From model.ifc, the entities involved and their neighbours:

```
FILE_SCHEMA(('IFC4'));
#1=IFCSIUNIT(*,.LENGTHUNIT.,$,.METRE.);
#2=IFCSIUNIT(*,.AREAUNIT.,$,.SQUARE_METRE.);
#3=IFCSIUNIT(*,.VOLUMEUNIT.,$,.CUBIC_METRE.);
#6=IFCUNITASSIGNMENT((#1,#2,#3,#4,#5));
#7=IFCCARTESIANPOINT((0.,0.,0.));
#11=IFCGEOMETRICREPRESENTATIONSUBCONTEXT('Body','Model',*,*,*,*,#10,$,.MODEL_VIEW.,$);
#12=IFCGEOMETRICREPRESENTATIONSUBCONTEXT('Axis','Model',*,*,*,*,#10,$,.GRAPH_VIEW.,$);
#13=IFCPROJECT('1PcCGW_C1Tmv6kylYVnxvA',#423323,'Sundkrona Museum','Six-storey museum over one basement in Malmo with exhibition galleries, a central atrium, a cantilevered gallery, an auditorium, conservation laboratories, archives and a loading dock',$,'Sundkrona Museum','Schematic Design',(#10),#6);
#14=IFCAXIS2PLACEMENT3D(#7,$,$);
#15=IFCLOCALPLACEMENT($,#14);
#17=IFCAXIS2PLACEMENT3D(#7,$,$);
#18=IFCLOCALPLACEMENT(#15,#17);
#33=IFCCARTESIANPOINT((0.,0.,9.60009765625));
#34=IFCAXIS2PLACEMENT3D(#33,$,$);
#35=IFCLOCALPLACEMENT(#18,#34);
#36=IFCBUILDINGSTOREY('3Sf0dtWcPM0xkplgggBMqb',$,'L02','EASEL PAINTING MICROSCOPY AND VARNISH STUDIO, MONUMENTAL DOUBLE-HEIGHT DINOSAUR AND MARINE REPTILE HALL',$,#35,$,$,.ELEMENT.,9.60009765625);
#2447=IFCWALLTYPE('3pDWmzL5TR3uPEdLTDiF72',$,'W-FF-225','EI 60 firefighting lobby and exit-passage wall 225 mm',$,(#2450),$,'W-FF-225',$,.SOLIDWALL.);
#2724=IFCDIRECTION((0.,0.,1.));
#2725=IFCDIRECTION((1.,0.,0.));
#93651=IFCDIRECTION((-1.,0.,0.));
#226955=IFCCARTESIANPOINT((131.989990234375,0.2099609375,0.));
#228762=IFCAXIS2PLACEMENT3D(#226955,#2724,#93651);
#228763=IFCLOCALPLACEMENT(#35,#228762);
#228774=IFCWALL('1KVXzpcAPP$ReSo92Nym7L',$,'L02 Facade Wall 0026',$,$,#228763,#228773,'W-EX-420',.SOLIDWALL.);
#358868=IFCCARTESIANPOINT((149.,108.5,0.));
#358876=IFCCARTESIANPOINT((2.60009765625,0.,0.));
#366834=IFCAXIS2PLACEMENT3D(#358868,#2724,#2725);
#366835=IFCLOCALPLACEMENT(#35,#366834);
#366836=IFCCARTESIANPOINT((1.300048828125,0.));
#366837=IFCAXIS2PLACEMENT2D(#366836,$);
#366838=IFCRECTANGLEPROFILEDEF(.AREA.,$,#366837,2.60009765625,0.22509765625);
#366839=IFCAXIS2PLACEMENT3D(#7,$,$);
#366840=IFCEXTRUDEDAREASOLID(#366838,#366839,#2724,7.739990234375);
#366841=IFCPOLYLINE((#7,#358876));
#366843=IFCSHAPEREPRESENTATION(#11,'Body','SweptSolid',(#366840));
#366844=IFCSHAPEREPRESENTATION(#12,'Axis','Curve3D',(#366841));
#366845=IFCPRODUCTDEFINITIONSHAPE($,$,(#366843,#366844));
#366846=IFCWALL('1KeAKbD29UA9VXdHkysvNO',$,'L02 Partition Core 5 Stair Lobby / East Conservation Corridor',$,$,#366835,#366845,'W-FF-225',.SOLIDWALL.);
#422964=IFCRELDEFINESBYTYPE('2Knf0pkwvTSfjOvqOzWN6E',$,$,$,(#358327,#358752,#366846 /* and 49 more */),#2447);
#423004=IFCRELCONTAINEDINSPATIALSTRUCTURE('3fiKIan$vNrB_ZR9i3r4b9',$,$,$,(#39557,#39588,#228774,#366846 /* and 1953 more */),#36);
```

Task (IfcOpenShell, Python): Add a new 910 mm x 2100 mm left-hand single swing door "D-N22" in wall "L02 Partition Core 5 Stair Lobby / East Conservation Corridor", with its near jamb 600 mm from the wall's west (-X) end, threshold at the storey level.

```python
import numpy as np
import ifcopenshell
import ifcopenshell.api.feature
import ifcopenshell.api.geometry
import ifcopenshell.api.root
import ifcopenshell.api.spatial
import ifcopenshell.geom
import ifcopenshell.util.element
import ifcopenshell.util.placement
import ifcopenshell.util.representation
import ifcopenshell.util.shape
import ifcopenshell.util.unit

model = ifcopenshell.open("model.ifc")
unit_scale = ifcopenshell.util.unit.calculate_unit_scale(model)
settings = ifcopenshell.geom.settings()


def volume(element):
    """Net volume in cubic metres, openings subtracted."""
    shape = ifcopenshell.geom.create_shape(settings, element)
    return ifcopenshell.util.shape.get_volume(shape.geometry)


wall = model.by_guid("1KeAKbD29UA9VXdHkysvNO")
storey = ifcopenshell.util.element.get_container(wall, ifc_class="IfcBuildingStorey")
context = ifcopenshell.util.representation.get_context(model, "Model", "Body", "MODEL_VIEW")
before = volume(wall)

width, height, from_end, sill = 0.91, 2.1, 0.6, 0.0  # metres

# The wall runs along its own X axis, and the end named is its -X end.
wall_shape = ifcopenshell.geom.create_shape(settings, wall)
x, y, z = ifcopenshell.util.shape.get_vertices(wall_shape.geometry).T
start = x.min() + from_end
face, thickness = float(y.min()), float(y.max() - y.min())
wall_matrix = ifcopenshell.util.placement.get_local_placement(wall.ObjectPlacement)
level = ifcopenshell.util.placement.get_local_placement(storey.ObjectPlacement)[2, 3]


def in_wall(x, y):
    """Placement at x, y metres in the wall's axes, at sill height."""
    matrix = wall_matrix.copy()
    matrix[:, 3] = wall_matrix @ np.array([x / unit_scale, y / unit_scale, 0.0, 1.0])
    matrix[2, 3] = level + sill / unit_scale
    return matrix


# Opening: a box that overshoots both wall faces by 50 mm.
opening = ifcopenshell.api.root.create_entity(model, ifc_class="IfcOpeningElement", predefined_type="OPENING")
box = ifcopenshell.api.geometry.add_wall_representation(
    model, context=context, length=width, height=height, thickness=thickness + 0.1
)
ifcopenshell.api.geometry.assign_representation(model, product=opening, representation=box)
ifcopenshell.api.geometry.edit_object_placement(model, product=opening, matrix=in_wall(start, face - 0.05), is_si=False)
ifcopenshell.api.feature.add_feature(model, feature=opening, element=wall)

door = ifcopenshell.api.root.create_entity(model, ifc_class="IfcDoor", name="D-N22", predefined_type="DOOR")
door.OverallWidth, door.OverallHeight = width / unit_scale, height / unit_scale
door.OperationType = "SINGLE_SWING_LEFT"
body = ifcopenshell.api.geometry.add_door_representation(
    model,
    context=context,
    overall_width=door.OverallWidth,
    overall_height=door.OverallHeight,
    operation_type="SINGLE_SWING_LEFT",
    lining_properties={"LiningDepth": thickness / unit_scale, "ThresholdDepth": thickness / unit_scale},
)
ifcopenshell.api.geometry.assign_representation(model, product=door, representation=body)
ifcopenshell.api.spatial.assign_container(model, products=[door], relating_structure=storey)
ifcopenshell.api.feature.add_filling(model, opening=opening, element=door)

# The lining spans the wall, so the door starts at the wall face.
ifcopenshell.api.geometry.edit_object_placement(model, product=door, matrix=in_wall(start, face), is_si=False)

after = volume(wall)

print(f"wall volume {before:.3f} -> {after:.3f} m3")

model.write("model-out.ifc")
```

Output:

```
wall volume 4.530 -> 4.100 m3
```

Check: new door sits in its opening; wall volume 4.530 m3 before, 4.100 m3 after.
